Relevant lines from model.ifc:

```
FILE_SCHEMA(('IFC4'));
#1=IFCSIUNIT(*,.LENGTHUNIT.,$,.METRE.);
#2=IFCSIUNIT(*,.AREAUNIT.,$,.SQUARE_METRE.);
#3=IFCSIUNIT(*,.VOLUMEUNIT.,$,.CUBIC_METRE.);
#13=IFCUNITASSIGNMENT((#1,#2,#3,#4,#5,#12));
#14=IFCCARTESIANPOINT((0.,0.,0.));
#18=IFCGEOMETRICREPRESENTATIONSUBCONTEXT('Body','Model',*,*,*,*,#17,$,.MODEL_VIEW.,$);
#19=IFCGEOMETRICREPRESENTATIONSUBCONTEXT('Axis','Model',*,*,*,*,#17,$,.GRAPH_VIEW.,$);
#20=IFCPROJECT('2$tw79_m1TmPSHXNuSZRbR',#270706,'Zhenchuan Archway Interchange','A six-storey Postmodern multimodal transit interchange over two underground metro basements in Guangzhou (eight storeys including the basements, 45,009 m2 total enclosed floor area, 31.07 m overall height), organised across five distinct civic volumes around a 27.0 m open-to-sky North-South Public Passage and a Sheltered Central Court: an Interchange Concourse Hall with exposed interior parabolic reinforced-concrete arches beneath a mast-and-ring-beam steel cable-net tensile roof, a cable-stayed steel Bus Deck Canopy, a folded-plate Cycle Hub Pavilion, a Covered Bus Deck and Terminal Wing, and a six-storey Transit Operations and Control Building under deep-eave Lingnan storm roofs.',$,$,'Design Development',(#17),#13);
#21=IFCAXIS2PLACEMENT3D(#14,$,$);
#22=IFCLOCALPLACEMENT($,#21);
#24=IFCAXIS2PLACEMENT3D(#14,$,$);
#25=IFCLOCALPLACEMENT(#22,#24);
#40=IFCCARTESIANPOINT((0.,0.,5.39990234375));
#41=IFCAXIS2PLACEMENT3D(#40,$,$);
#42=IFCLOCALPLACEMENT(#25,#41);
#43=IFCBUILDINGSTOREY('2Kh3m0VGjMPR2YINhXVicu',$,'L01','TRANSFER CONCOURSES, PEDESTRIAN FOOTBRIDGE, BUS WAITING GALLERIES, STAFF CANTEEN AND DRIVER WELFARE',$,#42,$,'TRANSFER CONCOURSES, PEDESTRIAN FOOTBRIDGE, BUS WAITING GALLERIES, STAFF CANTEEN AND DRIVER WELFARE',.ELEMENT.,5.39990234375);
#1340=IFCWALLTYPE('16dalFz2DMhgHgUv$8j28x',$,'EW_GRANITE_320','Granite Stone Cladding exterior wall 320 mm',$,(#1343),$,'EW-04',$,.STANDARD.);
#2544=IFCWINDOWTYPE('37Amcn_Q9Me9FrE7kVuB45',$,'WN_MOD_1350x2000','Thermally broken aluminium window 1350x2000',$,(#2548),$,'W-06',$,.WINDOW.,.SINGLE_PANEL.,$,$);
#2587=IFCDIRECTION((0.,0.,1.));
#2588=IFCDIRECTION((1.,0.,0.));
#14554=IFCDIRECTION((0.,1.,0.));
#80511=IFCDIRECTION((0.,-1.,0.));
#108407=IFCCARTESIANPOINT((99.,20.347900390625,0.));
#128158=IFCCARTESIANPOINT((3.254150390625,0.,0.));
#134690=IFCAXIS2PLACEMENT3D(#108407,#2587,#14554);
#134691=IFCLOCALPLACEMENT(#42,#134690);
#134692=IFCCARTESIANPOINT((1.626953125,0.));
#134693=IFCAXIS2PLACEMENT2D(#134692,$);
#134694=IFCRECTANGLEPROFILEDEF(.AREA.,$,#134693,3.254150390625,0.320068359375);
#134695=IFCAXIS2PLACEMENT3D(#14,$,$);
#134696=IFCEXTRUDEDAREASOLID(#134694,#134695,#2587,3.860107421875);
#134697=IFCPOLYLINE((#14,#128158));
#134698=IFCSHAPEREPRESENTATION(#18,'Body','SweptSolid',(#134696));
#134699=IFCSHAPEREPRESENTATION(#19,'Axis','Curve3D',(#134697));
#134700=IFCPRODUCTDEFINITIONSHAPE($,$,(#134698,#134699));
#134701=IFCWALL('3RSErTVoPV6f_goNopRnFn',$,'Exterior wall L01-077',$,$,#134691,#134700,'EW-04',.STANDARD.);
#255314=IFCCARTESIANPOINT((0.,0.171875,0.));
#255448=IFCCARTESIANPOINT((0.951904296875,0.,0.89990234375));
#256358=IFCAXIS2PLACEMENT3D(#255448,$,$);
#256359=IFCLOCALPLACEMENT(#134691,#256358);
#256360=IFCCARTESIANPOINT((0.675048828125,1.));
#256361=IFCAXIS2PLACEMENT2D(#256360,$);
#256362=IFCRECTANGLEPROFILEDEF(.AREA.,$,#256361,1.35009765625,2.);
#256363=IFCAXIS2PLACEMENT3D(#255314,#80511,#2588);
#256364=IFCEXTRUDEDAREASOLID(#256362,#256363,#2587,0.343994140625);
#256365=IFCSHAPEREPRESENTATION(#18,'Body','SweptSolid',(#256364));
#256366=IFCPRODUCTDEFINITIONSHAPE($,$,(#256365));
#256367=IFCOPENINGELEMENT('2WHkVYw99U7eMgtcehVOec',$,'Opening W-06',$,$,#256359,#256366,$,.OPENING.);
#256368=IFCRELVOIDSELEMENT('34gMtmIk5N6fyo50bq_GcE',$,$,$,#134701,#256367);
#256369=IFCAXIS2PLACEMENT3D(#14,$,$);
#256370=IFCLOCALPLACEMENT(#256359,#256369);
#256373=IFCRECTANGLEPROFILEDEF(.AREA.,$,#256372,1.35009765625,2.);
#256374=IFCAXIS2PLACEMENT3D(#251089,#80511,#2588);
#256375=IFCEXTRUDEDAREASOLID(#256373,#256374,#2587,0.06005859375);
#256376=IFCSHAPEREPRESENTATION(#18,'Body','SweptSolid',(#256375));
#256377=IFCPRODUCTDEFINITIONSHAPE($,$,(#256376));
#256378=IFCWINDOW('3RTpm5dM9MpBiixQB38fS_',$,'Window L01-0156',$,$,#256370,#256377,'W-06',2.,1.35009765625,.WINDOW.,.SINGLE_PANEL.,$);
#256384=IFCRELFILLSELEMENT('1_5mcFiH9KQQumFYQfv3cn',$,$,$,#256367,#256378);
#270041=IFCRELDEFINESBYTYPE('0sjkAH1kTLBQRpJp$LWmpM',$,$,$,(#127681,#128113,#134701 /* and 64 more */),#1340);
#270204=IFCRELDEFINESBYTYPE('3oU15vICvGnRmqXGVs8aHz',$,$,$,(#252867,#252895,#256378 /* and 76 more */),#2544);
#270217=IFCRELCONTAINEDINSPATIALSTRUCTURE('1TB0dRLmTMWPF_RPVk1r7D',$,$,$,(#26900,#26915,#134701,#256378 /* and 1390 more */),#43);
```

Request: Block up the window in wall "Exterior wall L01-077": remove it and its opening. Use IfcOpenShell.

```python
import ifcopenshell
import ifcopenshell.api.feature
import ifcopenshell.api.root
import ifcopenshell.geom
import ifcopenshell.util.shape

model = ifcopenshell.open("model.ifc")
settings = ifcopenshell.geom.settings()


def volume(element):
    """Net volume in cubic metres, openings subtracted."""
    shape = ifcopenshell.geom.create_shape(settings, element)
    return ifcopenshell.util.shape.get_volume(shape.geometry)


window = model.by_id(256378)
opening = window.FillsVoids[0].RelatingOpeningElement
wall = opening.VoidsElements[0].RelatingBuildingElement
before = volume(wall)

ifcopenshell.api.root.remove_product(model, product=window)
ifcopenshell.api.feature.remove_feature(model, feature=opening)

after = volume(wall)

print(f"wall volume {before:.3f} -> {after:.3f} m3")

model.write("model_rev.ifc")
```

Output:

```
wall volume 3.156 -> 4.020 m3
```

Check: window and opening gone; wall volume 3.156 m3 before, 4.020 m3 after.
